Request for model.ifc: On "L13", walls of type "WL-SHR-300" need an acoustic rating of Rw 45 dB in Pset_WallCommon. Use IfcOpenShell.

First a look at what the model holds.

```python
import ifcopenshell
import ifcopenshell.util.element

model = ifcopenshell.open("model.ifc")
print(model.schema)
storey = next(s for s in model.by_type("IfcBuildingStorey") if s.Name == "L13")
walls = [e for e in ifcopenshell.util.element.get_decomposition(storey) if e.is_a("IfcWall")]
seen = {}
for e in walls:
    element_type = ifcopenshell.util.element.get_type(e)
    key = (element_type.Name if element_type != e and element_type else None, ifcopenshell.util.element.get_pset(e, "Pset_WallCommon", "AcousticRating"))
    seen[key] = seen.get(key, 0) + 1
for (name, value), count in sorted(seen.items(), key=str):
    print(count, "x", name, "|", value)
```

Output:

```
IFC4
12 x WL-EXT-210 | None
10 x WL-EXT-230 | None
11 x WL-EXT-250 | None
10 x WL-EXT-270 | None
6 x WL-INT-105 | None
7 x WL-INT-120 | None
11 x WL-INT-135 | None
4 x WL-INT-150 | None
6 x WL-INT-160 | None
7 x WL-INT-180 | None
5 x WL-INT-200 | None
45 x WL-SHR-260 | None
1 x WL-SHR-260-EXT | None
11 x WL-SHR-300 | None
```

```python
import ifcopenshell
import ifcopenshell.api.pset
import ifcopenshell.util.element

model = ifcopenshell.open("model.ifc")

storey = next(s for s in model.by_type("IfcBuildingStorey") if s.Name == "L13")
walls = [e for e in ifcopenshell.util.element.get_decomposition(storey) if e.is_a("IfcWall")]

count = 0
for e in walls:
    element_type = ifcopenshell.util.element.get_type(e)
    if element_type in (None, e) or element_type.Name != "WL-SHR-300":
        continue
    # add_pset returns the element's existing set when there is one.
    pset = ifcopenshell.api.pset.add_pset(model, product=e, name="Pset_WallCommon")
    ifcopenshell.api.pset.edit_pset(model, pset=pset, properties={"AcousticRating": "Rw 45 dB"})
    count += 1

print(count, "walls updated")

model.write("model-out.ifc")
```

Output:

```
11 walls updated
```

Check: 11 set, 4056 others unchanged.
